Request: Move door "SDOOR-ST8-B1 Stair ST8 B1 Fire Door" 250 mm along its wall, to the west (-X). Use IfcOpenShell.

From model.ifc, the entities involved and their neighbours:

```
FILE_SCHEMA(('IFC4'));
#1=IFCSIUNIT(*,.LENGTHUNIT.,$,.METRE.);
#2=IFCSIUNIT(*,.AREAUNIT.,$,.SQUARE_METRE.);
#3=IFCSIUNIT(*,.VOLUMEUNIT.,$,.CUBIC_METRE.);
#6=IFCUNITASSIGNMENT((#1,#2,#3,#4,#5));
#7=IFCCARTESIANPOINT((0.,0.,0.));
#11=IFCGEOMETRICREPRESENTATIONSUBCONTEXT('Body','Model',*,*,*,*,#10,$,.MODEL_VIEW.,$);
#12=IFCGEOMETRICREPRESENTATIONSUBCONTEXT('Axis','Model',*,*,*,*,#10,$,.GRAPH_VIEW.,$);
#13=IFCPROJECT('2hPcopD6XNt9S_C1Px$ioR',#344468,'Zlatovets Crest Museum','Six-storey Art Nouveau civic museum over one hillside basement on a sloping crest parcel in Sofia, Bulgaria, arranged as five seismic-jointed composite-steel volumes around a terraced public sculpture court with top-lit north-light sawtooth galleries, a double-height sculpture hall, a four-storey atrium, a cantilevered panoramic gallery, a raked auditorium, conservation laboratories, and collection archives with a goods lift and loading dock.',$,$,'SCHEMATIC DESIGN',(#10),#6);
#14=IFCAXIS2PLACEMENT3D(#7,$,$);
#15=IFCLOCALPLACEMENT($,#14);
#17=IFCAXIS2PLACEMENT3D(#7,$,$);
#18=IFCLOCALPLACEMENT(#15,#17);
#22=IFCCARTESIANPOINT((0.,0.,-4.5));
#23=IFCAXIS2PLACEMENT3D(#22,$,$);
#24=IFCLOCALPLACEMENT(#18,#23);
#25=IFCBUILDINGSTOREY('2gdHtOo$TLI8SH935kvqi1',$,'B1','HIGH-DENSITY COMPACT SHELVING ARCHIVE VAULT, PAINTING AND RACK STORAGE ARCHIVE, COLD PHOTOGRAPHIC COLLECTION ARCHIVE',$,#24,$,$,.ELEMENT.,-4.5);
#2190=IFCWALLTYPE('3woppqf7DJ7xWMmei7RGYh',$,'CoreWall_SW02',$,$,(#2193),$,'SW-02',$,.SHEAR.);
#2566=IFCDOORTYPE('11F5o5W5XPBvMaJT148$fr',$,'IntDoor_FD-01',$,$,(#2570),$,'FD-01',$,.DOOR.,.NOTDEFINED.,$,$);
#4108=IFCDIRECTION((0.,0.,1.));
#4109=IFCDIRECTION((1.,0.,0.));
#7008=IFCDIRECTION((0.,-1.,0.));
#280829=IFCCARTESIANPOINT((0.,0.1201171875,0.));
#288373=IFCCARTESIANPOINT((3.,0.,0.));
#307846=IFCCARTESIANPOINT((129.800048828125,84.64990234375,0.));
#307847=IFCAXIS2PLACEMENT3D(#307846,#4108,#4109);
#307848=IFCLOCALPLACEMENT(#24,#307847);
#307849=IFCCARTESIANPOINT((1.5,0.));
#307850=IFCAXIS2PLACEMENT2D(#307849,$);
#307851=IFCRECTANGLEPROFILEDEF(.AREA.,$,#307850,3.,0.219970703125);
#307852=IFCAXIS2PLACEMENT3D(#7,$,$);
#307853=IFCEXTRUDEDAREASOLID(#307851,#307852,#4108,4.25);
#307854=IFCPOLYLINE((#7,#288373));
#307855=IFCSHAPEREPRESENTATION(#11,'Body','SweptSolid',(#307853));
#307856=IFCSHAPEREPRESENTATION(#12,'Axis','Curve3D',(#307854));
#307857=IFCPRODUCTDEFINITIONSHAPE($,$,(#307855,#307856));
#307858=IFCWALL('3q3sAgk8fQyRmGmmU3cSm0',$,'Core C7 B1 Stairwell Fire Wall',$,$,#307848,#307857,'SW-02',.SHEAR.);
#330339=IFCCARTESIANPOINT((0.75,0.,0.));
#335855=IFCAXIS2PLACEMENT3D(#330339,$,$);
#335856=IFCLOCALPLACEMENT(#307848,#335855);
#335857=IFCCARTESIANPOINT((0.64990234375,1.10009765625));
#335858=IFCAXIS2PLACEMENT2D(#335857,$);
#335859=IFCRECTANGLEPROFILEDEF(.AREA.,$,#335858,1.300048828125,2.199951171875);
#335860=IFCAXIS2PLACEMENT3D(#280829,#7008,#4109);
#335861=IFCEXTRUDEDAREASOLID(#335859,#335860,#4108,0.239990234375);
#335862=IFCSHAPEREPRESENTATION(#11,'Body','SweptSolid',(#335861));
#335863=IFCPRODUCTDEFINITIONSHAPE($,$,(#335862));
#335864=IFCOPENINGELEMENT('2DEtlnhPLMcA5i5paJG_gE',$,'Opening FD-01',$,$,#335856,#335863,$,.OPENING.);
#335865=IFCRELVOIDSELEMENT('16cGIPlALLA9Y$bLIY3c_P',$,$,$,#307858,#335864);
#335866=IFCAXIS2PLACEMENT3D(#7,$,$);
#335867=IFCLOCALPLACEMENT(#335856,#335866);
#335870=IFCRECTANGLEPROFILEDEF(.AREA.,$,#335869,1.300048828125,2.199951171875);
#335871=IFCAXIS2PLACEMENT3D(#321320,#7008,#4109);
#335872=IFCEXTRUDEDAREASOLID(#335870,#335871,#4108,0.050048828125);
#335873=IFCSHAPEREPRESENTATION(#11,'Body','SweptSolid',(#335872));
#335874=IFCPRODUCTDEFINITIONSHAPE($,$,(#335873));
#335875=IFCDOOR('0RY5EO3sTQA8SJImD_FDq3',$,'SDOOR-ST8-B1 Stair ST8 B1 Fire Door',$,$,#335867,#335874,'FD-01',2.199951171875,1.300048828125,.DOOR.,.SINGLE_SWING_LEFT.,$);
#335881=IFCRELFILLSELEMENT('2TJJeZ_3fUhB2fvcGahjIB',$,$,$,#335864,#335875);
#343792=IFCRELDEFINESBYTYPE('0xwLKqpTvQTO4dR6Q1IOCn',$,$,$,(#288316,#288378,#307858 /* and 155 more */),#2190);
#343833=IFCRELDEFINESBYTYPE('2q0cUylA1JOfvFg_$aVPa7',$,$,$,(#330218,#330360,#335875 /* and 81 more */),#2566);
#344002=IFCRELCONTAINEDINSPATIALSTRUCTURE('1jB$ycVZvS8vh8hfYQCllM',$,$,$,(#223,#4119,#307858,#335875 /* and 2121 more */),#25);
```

```python
import ifcopenshell
import ifcopenshell.api.geometry
import ifcopenshell.util.placement

model = ifcopenshell.open("model.ifc")

door = model.by_id(335875)
opening = door.FillsVoids[0].RelatingOpeningElement
wall = opening.VoidsElements[0].RelatingBuildingElement

wall_matrix = ifcopenshell.util.placement.get_local_placement(wall.ObjectPlacement)
shift = wall_matrix[:3, 0] * -0.25
before = ifcopenshell.util.placement.get_local_placement(door.ObjectPlacement)[:3, 3].copy()

# The door is placed relative to its opening, so it follows when the opening moves.
matrix = ifcopenshell.util.placement.get_local_placement(opening.ObjectPlacement)
matrix[:3, 3] += shift
ifcopenshell.api.geometry.edit_object_placement(
    model, product=opening, matrix=matrix, is_si=False, should_transform_children=True
)

after = ifcopenshell.util.placement.get_local_placement(door.ObjectPlacement)[:3, 3]
print("door moved by", (after - before).round(3) + 0.0)

model.write("model_edited.ifc")
```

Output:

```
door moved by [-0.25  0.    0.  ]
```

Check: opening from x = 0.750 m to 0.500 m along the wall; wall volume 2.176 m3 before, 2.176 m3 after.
